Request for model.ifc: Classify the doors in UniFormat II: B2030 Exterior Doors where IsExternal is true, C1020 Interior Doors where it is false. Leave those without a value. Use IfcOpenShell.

First a look at what the model holds.

```python
import ifcopenshell
import ifcopenshell.util.element

model = ifcopenshell.open("model.ifc")
print(model.schema)
print("classifications:", [c.Name for c in model.by_type("IfcClassification")])
values = [ifcopenshell.util.element.get_pset(e, "Pset_DoorCommon", "IsExternal") for e in model.by_type("IfcDoor")]
for value in (True, False, None):
    print("IsExternal", value, values.count(value))
```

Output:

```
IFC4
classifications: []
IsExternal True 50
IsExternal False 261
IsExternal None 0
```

```python
import ifcopenshell
import ifcopenshell.api.classification
import ifcopenshell.util.element

model = ifcopenshell.open("model.ifc")

system = ifcopenshell.api.classification.add_classification(model, classification="UniFormat II")

doors = model.by_type("IfcDoor")
external = {e: ifcopenshell.util.element.get_pset(e, "Pset_DoorCommon", "IsExternal") for e in doors}
for flag, code, name in ((True, "B2030", "Exterior Doors"), (False, "C1020", "Interior Doors")):
    products = [e for e in doors if external[e] is flag]
    ifcopenshell.api.classification.add_reference(
        model, products=products, classification=system, identification=code, name=name
    )
    print(code, len(products))

model.write("model_v2.ifc")
```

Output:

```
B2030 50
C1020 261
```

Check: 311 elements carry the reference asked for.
